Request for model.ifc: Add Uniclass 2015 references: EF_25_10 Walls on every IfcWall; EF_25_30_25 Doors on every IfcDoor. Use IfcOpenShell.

First a look at what the model holds.

```python
import ifcopenshell

model = ifcopenshell.open("model.ifc")
print(model.schema)
print("classifications:", [c.Name for c in model.by_type("IfcClassification")])
for ifc_class in ("IfcDoor", "IfcRoof", "IfcStair", "IfcWall", "IfcWindow"):
    print(ifc_class, len(model.by_type(ifc_class)))
```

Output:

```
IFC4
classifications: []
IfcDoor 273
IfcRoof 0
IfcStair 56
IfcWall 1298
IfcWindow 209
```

```python
import ifcopenshell
import ifcopenshell.api.classification

model = ifcopenshell.open("model.ifc")

system = ifcopenshell.api.classification.add_classification(model, classification="Uniclass 2015")

codes = {
    "IfcWall": ("EF_25_10", "Walls"),
    "IfcDoor": ("EF_25_30_25", "Doors"),
}
for ifc_class, (code, name) in codes.items():
    products = model.by_type(ifc_class)
    ifcopenshell.api.classification.add_reference(
        model, products=products, classification=system, identification=code, name=name
    )
    print(code, len(products))

model.write("model-out.ifc")
```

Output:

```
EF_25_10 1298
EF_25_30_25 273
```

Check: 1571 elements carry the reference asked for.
